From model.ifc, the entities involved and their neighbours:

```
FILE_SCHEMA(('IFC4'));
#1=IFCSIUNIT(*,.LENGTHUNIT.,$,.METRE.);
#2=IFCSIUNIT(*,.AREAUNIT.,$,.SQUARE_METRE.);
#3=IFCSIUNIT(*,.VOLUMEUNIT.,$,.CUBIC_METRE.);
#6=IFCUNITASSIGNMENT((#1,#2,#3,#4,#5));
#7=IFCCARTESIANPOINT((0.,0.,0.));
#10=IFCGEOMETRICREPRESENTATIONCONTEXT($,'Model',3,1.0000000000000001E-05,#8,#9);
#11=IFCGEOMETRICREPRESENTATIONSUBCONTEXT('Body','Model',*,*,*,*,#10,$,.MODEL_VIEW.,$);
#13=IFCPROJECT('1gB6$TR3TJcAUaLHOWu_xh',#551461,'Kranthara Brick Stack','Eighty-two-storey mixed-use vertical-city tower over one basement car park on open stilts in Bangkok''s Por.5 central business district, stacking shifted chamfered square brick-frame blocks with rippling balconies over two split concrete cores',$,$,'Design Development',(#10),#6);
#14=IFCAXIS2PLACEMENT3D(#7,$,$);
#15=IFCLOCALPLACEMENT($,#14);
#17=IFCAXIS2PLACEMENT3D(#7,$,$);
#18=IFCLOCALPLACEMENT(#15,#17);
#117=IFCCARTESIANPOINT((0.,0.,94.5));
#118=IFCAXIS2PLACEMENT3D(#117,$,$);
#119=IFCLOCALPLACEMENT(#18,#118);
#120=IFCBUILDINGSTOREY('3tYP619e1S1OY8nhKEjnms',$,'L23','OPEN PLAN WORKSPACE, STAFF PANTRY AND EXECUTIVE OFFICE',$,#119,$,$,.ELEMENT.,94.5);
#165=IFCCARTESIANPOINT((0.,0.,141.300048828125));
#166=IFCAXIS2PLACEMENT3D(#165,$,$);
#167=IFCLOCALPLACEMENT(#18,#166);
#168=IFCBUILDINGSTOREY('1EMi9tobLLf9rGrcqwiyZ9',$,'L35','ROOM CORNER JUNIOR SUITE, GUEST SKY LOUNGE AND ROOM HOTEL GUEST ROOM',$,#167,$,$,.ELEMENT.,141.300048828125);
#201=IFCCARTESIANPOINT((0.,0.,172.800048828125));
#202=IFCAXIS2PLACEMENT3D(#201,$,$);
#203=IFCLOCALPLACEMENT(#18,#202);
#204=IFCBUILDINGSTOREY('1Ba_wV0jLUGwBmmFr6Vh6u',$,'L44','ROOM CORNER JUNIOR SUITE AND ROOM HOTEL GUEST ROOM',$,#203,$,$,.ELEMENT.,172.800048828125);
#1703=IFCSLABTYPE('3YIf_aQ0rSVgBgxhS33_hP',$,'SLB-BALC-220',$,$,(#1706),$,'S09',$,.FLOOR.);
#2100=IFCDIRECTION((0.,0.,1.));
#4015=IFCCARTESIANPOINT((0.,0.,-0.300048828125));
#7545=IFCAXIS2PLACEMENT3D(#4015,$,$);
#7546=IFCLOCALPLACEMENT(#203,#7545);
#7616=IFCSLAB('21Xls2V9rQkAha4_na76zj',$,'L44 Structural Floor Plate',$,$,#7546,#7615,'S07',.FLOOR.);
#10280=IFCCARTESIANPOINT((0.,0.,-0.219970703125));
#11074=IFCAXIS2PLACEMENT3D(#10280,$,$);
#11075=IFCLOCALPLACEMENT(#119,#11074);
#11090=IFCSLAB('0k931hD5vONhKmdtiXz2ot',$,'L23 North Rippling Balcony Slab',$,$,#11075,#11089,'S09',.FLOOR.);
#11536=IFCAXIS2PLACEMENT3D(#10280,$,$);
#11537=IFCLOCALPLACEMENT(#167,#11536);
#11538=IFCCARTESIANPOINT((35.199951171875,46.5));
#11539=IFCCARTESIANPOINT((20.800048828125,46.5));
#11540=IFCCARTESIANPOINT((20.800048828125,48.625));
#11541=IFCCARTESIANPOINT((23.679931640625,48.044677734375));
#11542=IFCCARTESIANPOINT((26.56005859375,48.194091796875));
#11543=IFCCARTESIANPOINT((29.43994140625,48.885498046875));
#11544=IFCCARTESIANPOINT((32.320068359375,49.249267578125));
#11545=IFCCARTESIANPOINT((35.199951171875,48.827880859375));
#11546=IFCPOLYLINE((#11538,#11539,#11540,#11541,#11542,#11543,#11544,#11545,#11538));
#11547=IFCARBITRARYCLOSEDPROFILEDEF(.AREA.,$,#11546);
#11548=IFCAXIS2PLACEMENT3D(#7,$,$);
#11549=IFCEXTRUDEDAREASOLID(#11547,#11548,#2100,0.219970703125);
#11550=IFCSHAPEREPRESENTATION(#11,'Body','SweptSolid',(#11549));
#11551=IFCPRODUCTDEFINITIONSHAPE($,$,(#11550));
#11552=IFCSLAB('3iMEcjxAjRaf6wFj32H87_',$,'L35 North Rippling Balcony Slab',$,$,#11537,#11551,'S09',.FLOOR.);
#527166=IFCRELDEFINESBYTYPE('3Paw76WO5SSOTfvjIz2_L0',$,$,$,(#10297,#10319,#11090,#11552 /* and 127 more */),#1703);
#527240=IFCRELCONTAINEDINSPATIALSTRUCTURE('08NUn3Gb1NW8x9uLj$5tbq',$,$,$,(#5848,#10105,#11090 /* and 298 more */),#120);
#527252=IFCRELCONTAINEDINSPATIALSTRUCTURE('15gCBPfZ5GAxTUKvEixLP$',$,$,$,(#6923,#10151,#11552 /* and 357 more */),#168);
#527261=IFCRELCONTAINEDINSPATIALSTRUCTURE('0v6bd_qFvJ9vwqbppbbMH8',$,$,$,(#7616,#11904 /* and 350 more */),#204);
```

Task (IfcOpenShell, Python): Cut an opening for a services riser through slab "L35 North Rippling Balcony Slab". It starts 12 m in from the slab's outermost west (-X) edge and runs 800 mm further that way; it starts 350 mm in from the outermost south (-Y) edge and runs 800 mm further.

```python
import numpy as np
import ifcopenshell
import ifcopenshell.api.feature
import ifcopenshell.api.geometry
import ifcopenshell.api.root
import ifcopenshell.geom
import ifcopenshell.util.placement
import ifcopenshell.util.representation
import ifcopenshell.util.shape
import ifcopenshell.util.unit

model = ifcopenshell.open("model.ifc")
unit_scale = ifcopenshell.util.unit.calculate_unit_scale(model)
settings = ifcopenshell.geom.settings()


def volume(element):
    """Net volume in cubic metres, openings subtracted."""
    shape = ifcopenshell.geom.create_shape(settings, element)
    return ifcopenshell.util.shape.get_volume(shape.geometry)


slab = model.by_guid("3iMEcjxAjRaf6wFj32H87_")
before = volume(slab)

# Extent in the slab's own axes, in metres. The edges named are its -X and -Y sides.
slab_shape = ifcopenshell.geom.create_shape(settings, slab)
vertices = ifcopenshell.util.shape.get_vertices(slab_shape.geometry)
x_min, y_min, bottom = vertices.min(axis=0)
top = vertices[:, 2].max()

opening = ifcopenshell.api.root.create_entity(model, ifc_class="IfcOpeningElement", name="Services riser opening", predefined_type="OPENING")
context = ifcopenshell.util.representation.get_context(model, "Model", "Body", "MODEL_VIEW")
width, depth = 0.8, 0.8
outline = [(0.0, 0.0), (width, 0.0), (width, depth), (0.0, depth), (0.0, 0.0)]
# Overshoot both faces by 50 mm so the cut is clean.
shape = ifcopenshell.api.geometry.add_slab_representation(
    model, context=context, depth=top - bottom + 0.1, polyline=outline
)
ifcopenshell.api.geometry.assign_representation(model, product=opening, representation=shape)

matrix = ifcopenshell.util.placement.get_local_placement(slab.ObjectPlacement)
matrix[:, 3] = matrix @ np.append(np.array([x_min + 12, y_min + 0.35, bottom - 0.05]) / unit_scale, 1.0)
ifcopenshell.api.geometry.edit_object_placement(model, product=opening, matrix=matrix, is_si=False)
ifcopenshell.api.feature.add_feature(model, feature=opening, element=slab)

after = volume(slab)

print(f"slab volume {before:.3f} -> {after:.3f} m3")

model.write("model_rev.ifc")
```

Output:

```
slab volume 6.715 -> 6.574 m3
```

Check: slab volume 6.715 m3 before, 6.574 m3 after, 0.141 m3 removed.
